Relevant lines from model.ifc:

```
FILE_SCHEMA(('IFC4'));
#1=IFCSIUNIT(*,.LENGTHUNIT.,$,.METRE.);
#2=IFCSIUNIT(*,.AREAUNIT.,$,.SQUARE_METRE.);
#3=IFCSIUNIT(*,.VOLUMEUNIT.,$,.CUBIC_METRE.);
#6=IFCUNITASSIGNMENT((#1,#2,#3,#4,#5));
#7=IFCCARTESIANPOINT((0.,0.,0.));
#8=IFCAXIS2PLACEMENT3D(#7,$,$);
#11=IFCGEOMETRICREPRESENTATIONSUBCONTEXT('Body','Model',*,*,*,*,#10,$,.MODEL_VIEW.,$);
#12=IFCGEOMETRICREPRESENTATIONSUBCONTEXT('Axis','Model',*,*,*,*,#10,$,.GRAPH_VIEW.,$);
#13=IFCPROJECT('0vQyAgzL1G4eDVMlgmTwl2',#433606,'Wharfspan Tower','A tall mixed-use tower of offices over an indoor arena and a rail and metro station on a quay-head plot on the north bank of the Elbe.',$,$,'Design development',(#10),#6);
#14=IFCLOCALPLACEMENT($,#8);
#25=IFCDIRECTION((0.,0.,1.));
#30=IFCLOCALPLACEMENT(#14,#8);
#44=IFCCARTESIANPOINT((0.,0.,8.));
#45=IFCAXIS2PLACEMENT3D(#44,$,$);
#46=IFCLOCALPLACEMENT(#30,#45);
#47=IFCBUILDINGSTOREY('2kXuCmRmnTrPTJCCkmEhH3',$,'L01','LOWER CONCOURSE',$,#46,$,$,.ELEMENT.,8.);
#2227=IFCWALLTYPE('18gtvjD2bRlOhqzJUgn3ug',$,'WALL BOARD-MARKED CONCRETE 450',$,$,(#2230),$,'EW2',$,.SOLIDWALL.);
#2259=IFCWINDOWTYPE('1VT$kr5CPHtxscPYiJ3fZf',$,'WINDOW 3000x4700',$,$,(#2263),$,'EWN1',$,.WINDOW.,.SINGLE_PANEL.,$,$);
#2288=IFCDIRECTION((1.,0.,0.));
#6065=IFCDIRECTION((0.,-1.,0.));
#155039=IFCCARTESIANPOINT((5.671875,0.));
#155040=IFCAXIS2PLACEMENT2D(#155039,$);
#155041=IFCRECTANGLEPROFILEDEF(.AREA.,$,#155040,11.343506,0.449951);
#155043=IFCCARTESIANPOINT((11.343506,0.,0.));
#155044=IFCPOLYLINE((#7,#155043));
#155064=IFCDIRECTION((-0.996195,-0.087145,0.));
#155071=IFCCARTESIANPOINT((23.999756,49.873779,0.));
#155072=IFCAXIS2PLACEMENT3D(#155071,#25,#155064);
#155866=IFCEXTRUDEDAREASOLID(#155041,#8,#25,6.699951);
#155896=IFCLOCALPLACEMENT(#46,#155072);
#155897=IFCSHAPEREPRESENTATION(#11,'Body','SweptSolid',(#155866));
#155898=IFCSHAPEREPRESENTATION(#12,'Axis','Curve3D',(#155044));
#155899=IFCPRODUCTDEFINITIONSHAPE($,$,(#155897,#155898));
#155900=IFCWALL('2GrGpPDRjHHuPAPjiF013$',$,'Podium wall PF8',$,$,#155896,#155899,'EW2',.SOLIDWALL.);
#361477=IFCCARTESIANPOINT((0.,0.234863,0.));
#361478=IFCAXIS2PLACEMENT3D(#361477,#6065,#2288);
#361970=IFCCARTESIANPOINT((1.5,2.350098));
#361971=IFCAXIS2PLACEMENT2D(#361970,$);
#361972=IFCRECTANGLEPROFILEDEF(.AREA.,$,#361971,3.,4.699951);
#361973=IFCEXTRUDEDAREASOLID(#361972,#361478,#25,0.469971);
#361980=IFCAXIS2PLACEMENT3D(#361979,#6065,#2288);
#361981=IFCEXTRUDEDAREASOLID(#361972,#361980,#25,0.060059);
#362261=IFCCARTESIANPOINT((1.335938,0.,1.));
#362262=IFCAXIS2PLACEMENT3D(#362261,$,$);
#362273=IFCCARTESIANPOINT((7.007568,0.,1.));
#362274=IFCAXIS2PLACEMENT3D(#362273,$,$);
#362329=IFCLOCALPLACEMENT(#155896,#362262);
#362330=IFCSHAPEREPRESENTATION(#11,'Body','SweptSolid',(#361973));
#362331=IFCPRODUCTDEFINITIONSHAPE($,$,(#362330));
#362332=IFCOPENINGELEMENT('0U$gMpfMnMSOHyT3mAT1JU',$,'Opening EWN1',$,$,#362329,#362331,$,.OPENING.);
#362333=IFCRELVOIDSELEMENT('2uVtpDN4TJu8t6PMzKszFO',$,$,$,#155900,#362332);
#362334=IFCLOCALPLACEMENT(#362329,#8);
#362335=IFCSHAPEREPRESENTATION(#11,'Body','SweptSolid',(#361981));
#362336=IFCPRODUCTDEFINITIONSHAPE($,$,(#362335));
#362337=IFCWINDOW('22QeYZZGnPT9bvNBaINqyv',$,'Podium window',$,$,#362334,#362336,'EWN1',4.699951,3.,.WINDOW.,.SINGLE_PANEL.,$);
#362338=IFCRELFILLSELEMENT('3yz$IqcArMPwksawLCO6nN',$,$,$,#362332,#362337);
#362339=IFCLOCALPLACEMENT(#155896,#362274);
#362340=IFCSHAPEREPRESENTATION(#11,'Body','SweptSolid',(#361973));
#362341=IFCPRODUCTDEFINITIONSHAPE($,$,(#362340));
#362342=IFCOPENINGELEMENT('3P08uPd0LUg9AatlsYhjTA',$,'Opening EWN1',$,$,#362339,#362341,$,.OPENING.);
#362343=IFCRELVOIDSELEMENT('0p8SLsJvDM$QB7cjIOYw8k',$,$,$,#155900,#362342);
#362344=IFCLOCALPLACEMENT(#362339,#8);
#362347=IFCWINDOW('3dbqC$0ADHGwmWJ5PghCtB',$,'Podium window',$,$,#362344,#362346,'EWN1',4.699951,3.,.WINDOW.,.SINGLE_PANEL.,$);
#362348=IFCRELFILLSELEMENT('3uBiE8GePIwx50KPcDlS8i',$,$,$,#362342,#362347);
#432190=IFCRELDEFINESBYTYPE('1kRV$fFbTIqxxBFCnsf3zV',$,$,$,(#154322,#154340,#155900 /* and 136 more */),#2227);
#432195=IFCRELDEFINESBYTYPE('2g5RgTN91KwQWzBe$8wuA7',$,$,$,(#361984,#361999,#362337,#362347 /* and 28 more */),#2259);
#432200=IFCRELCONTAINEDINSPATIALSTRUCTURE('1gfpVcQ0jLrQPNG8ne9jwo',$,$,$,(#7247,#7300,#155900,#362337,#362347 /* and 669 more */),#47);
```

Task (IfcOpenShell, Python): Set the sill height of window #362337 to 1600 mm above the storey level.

```python
import numpy as np
import ifcopenshell
import ifcopenshell.api.geometry
import ifcopenshell.geom
import ifcopenshell.util.element
import ifcopenshell.util.placement
import ifcopenshell.util.shape
import ifcopenshell.util.unit

model = ifcopenshell.open("model.ifc")
unit_scale = ifcopenshell.util.unit.calculate_unit_scale(model)

window = model.by_id(362337)
opening = window.FillsVoids[0].RelatingOpeningElement
storey = ifcopenshell.util.element.get_container(window, ifc_class="IfcBuildingStorey")
level = ifcopenshell.util.placement.get_local_placement(storey.ObjectPlacement)[2, 3]

# The opening's origin need not be at the sill, so measure its lowest point.
shape = ifcopenshell.geom.create_shape(ifcopenshell.geom.settings(), opening)
bottom = ifcopenshell.util.shape.get_shape_bottom_elevation(shape, shape.geometry) / unit_scale
dz = level + 1.6 - bottom

shift = np.array([0.0, 0.0, dz])
# The window is placed relative to its opening, so it follows when the opening moves.
matrix = ifcopenshell.util.placement.get_local_placement(opening.ObjectPlacement)
matrix[:3, 3] += shift
ifcopenshell.api.geometry.edit_object_placement(
    model, product=opening, matrix=matrix, is_si=False, should_transform_children=True
)

print(f"moved by {dz * unit_scale:+.3f} m")

model.write("model_rev.ifc")
```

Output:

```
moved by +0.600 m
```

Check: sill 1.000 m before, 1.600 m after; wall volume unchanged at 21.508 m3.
